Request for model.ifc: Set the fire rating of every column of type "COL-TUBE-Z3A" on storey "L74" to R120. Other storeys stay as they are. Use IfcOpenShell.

First a look at what the model holds.

```python
import ifcopenshell
import ifcopenshell.util.element

model = ifcopenshell.open("model.ifc")
print(model.schema)
storey = next(s for s in model.by_type("IfcBuildingStorey") if s.Name == "L74")
columns = [e for e in ifcopenshell.util.element.get_decomposition(storey) if e.is_a("IfcColumn")]
seen = {}
for e in columns:
    element_type = ifcopenshell.util.element.get_type(e)
    key = (element_type.Name if element_type != e and element_type else None, ifcopenshell.util.element.get_pset(e, "Pset_ColumnCommon", "FireRating"))
    seen[key] = seen.get(key, 0) + 1
for (name, value), count in sorted(seen.items(), key=str):
    print(count, "x", name, "|", value)
```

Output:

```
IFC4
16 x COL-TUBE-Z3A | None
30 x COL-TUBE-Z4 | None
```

```python
import ifcopenshell
import ifcopenshell.api.pset
import ifcopenshell.util.element

model = ifcopenshell.open("model.ifc")

storey = next(s for s in model.by_type("IfcBuildingStorey") if s.Name == "L74")
columns = [e for e in ifcopenshell.util.element.get_decomposition(storey) if e.is_a("IfcColumn")]

count = 0
for e in columns:
    element_type = ifcopenshell.util.element.get_type(e)
    if element_type in (None, e) or element_type.Name != "COL-TUBE-Z3A":
        continue
    found = ifcopenshell.util.element.get_pset(e, "Pset_ColumnCommon", should_inherit=False)
    if found:
        pset = model.by_id(found["id"])
        if len(ifcopenshell.util.element.get_elements_by_pset(pset)) > 1:
            pset = ifcopenshell.api.pset.unshare_pset(model, products=[e], pset=pset)[0]
    else:
        pset = ifcopenshell.api.pset.add_pset(model, product=e, name="Pset_ColumnCommon")
    ifcopenshell.api.pset.edit_pset(model, pset=pset, properties={"FireRating": "R120"})
    count += 1

print(count, "columns updated")

model.write("model_v2.ifc")
```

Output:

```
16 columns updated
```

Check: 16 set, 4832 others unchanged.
